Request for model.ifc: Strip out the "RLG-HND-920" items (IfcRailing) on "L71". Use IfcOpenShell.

First a look at what the model holds.

```python
import ifcopenshell
import ifcopenshell.util.element

model = ifcopenshell.open("model.ifc")
print(model.schema)
storey = next(s for s in model.by_type("IfcBuildingStorey") if s.Name == "L71")
railings = [e for e in ifcopenshell.util.element.get_decomposition(storey) if e.is_a("IfcRailing")]
seen = {}
for e in railings:
    element_type = ifcopenshell.util.element.get_type(e)
    name = element_type.Name if element_type not in (None, e) else None
    seen[name] = seen.get(name, 0) + 1
for name, count in sorted(seen.items(), key=str):
    print(count, "x", name)
```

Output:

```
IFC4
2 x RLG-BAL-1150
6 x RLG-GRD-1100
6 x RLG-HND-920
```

```python
import ifcopenshell
import ifcopenshell.api.root
import ifcopenshell.util.element

model = ifcopenshell.open("model.ifc")

storey = next(s for s in model.by_type("IfcBuildingStorey") if s.Name == "L71")
railings = [e for e in ifcopenshell.util.element.get_decomposition(storey) if e.is_a("IfcRailing")]
targets = [e for e in railings if (t := ifcopenshell.util.element.get_type(e)) not in (None, e) and t.Name == "RLG-HND-920"]

for e in targets:
    ifcopenshell.api.root.remove_product(model, product=e)
print(len(targets), "removed")

model.write("model_rev.ifc")
```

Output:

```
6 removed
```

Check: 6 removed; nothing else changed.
